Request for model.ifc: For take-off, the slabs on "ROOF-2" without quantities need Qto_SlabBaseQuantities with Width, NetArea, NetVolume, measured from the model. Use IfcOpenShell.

First a look at what the model holds.

```python
import ifcopenshell
import ifcopenshell.util.element
import ifcopenshell.util.unit

model = ifcopenshell.open("model.ifc")
print(model.schema)
for unit_type in ("LENGTHUNIT", "AREAUNIT", "VOLUMEUNIT"):
    print(unit_type, ifcopenshell.util.unit.calculate_unit_scale(model, unit_type))
storey = next(s for s in model.by_type("IfcBuildingStorey") if s.Name == "ROOF-2")
slabs = [e for e in ifcopenshell.util.element.get_decomposition(storey) if e.is_a("IfcSlab")]
for e in sorted(slabs, key=lambda e: e.id()):
    print(e.id(), e.is_a(), e.Name, list(ifcopenshell.util.element.get_psets(e, qtos_only=True)), sep=" | ")
```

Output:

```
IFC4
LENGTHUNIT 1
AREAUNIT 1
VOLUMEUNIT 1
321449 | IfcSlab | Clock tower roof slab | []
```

```python
import ifcopenshell
import ifcopenshell.api.pset
import ifcopenshell.geom
import ifcopenshell.util.element
import ifcopenshell.util.shape
import ifcopenshell.util.unit

model = ifcopenshell.open("model.ifc")
unit_scale = ifcopenshell.util.unit.calculate_unit_scale(model)
area_scale = ifcopenshell.util.unit.calculate_unit_scale(model, "AREAUNIT")
volume_scale = ifcopenshell.util.unit.calculate_unit_scale(model, "VOLUMEUNIT")
settings = ifcopenshell.geom.settings()

storey = next(s for s in model.by_type("IfcBuildingStorey") if s.Name == "ROOF-2")
slabs = [e for e in ifcopenshell.util.element.get_decomposition(storey) if e.is_a("IfcSlab")]

for e in sorted(slabs, key=lambda e: e.id()):
    if ifcopenshell.util.element.get_psets(e, qtos_only=True, should_inherit=False):
        continue
    # Geometry comes back in metres, in the element's own axes.
    shape = ifcopenshell.geom.create_shape(settings, e)
    values = {
        "Width": ifcopenshell.util.shape.get_z(shape.geometry) / unit_scale,
        "NetArea": ifcopenshell.util.shape.get_footprint_area(shape.geometry) / area_scale,
        "NetVolume": ifcopenshell.util.shape.get_volume(shape.geometry) / volume_scale,
    }
    qto = ifcopenshell.api.pset.add_qto(model, product=e, name="Qto_SlabBaseQuantities")
    ifcopenshell.api.pset.edit_qto(model, qto=qto, properties=values)
    print(e.id(), {k: round(v, 3) for k, v in values.items()})

model.write("model_updated.ifc")
```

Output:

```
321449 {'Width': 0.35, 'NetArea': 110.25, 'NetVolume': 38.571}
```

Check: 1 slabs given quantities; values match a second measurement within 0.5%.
